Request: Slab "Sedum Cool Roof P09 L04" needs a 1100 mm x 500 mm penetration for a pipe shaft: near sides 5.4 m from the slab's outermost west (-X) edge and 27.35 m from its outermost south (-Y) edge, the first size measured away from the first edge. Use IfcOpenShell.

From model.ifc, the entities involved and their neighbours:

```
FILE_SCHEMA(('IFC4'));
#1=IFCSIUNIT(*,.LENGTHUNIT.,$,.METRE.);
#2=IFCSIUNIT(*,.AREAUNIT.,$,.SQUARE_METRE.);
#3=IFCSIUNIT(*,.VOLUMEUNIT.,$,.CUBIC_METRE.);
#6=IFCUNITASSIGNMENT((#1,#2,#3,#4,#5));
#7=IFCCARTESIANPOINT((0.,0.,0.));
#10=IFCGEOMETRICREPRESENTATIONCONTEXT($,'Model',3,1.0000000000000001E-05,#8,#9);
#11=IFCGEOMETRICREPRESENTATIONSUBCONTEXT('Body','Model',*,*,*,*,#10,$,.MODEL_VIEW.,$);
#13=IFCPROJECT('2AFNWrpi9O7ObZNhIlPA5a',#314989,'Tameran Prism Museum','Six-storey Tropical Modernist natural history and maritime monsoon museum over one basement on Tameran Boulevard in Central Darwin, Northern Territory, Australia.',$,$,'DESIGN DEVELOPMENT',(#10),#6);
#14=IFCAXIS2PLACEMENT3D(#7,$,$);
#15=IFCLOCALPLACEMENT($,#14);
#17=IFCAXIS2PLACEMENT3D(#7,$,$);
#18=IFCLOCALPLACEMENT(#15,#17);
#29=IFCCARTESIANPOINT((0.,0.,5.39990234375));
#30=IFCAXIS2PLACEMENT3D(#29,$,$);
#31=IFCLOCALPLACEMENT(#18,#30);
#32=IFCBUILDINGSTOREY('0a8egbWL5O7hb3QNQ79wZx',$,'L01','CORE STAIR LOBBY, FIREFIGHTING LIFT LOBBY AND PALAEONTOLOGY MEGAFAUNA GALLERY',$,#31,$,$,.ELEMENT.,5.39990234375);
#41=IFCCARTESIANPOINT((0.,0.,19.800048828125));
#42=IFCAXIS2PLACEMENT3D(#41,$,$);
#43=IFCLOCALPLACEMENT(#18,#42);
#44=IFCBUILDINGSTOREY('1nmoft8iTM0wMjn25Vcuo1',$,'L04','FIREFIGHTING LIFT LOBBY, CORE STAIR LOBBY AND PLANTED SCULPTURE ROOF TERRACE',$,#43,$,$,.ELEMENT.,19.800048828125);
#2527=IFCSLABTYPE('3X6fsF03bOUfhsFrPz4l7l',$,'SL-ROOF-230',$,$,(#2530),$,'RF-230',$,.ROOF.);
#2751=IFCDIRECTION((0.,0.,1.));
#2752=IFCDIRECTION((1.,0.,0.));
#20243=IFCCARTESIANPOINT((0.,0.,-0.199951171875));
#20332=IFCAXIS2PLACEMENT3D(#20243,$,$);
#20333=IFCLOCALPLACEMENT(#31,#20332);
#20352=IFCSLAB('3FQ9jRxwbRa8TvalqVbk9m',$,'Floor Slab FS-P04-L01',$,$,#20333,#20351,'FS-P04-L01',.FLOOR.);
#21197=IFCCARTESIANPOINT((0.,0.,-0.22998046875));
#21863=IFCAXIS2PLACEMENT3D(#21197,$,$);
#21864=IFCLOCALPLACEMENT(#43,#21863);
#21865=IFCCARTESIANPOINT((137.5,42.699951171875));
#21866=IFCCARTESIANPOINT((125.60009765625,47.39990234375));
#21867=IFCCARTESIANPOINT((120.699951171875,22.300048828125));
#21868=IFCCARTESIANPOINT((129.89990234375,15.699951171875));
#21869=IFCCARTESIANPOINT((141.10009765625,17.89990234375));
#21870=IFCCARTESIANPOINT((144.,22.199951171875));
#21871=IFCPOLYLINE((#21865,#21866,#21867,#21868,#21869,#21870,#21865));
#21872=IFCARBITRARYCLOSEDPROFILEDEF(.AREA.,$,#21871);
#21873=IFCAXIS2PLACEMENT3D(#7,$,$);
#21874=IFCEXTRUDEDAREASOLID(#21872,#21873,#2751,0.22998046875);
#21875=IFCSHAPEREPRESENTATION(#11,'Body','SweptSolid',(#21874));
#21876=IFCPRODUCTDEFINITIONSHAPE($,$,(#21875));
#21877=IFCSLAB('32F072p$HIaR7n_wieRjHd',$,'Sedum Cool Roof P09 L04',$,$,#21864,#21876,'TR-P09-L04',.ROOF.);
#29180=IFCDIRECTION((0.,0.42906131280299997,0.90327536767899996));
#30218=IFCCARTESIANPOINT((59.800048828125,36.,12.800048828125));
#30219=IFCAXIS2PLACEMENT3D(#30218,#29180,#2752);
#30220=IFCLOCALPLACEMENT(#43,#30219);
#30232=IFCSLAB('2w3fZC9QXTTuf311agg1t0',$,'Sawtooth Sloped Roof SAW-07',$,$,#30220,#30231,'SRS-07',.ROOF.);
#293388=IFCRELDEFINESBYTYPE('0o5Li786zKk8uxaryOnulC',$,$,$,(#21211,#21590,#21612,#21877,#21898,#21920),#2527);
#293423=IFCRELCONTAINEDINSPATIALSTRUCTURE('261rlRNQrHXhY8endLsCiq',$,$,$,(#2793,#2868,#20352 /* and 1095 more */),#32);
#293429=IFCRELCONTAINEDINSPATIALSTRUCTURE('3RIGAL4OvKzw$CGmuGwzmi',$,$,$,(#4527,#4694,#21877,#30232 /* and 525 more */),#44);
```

```python
import numpy as np
import ifcopenshell
import ifcopenshell.api.feature
import ifcopenshell.api.geometry
import ifcopenshell.api.root
import ifcopenshell.geom
import ifcopenshell.util.placement
import ifcopenshell.util.representation
import ifcopenshell.util.shape
import ifcopenshell.util.unit

model = ifcopenshell.open("model.ifc")
unit_scale = ifcopenshell.util.unit.calculate_unit_scale(model)
settings = ifcopenshell.geom.settings()


def volume(element):
    """Net volume in cubic metres, openings subtracted."""
    shape = ifcopenshell.geom.create_shape(settings, element)
    return ifcopenshell.util.shape.get_volume(shape.geometry)


slab = model.by_guid("32F072p$HIaR7n_wieRjHd")
before = volume(slab)

# Extent in the slab's own axes, in metres. The edges named are its -X and -Y sides.
slab_shape = ifcopenshell.geom.create_shape(settings, slab)
vertices = ifcopenshell.util.shape.get_vertices(slab_shape.geometry)
x_min, y_min, bottom = vertices.min(axis=0)
top = vertices[:, 2].max()

opening = ifcopenshell.api.root.create_entity(model, ifc_class="IfcOpeningElement", name="Pipe shaft opening", predefined_type="OPENING")
context = ifcopenshell.util.representation.get_context(model, "Model", "Body", "MODEL_VIEW")
width, depth = 1.1, 0.5
outline = [(0.0, 0.0), (width, 0.0), (width, depth), (0.0, depth), (0.0, 0.0)]
# Overshoot both faces by 50 mm so the cut is clean.
shape = ifcopenshell.api.geometry.add_slab_representation(
    model, context=context, depth=top - bottom + 0.1, polyline=outline
)
ifcopenshell.api.geometry.assign_representation(model, product=opening, representation=shape)

matrix = ifcopenshell.util.placement.get_local_placement(slab.ObjectPlacement)
matrix[:, 3] = matrix @ np.append(np.array([x_min + 5.4, y_min + 27.35, bottom - 0.05]) / unit_scale, 1.0)
ifcopenshell.api.geometry.edit_object_placement(model, product=opening, matrix=matrix, is_si=False)
ifcopenshell.api.feature.add_feature(model, feature=opening, element=slab)

after = volume(slab)

print(f"slab volume {before:.3f} -> {after:.3f} m3")

model.write("model_v2.ifc")
```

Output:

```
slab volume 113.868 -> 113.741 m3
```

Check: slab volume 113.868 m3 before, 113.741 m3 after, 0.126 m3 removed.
